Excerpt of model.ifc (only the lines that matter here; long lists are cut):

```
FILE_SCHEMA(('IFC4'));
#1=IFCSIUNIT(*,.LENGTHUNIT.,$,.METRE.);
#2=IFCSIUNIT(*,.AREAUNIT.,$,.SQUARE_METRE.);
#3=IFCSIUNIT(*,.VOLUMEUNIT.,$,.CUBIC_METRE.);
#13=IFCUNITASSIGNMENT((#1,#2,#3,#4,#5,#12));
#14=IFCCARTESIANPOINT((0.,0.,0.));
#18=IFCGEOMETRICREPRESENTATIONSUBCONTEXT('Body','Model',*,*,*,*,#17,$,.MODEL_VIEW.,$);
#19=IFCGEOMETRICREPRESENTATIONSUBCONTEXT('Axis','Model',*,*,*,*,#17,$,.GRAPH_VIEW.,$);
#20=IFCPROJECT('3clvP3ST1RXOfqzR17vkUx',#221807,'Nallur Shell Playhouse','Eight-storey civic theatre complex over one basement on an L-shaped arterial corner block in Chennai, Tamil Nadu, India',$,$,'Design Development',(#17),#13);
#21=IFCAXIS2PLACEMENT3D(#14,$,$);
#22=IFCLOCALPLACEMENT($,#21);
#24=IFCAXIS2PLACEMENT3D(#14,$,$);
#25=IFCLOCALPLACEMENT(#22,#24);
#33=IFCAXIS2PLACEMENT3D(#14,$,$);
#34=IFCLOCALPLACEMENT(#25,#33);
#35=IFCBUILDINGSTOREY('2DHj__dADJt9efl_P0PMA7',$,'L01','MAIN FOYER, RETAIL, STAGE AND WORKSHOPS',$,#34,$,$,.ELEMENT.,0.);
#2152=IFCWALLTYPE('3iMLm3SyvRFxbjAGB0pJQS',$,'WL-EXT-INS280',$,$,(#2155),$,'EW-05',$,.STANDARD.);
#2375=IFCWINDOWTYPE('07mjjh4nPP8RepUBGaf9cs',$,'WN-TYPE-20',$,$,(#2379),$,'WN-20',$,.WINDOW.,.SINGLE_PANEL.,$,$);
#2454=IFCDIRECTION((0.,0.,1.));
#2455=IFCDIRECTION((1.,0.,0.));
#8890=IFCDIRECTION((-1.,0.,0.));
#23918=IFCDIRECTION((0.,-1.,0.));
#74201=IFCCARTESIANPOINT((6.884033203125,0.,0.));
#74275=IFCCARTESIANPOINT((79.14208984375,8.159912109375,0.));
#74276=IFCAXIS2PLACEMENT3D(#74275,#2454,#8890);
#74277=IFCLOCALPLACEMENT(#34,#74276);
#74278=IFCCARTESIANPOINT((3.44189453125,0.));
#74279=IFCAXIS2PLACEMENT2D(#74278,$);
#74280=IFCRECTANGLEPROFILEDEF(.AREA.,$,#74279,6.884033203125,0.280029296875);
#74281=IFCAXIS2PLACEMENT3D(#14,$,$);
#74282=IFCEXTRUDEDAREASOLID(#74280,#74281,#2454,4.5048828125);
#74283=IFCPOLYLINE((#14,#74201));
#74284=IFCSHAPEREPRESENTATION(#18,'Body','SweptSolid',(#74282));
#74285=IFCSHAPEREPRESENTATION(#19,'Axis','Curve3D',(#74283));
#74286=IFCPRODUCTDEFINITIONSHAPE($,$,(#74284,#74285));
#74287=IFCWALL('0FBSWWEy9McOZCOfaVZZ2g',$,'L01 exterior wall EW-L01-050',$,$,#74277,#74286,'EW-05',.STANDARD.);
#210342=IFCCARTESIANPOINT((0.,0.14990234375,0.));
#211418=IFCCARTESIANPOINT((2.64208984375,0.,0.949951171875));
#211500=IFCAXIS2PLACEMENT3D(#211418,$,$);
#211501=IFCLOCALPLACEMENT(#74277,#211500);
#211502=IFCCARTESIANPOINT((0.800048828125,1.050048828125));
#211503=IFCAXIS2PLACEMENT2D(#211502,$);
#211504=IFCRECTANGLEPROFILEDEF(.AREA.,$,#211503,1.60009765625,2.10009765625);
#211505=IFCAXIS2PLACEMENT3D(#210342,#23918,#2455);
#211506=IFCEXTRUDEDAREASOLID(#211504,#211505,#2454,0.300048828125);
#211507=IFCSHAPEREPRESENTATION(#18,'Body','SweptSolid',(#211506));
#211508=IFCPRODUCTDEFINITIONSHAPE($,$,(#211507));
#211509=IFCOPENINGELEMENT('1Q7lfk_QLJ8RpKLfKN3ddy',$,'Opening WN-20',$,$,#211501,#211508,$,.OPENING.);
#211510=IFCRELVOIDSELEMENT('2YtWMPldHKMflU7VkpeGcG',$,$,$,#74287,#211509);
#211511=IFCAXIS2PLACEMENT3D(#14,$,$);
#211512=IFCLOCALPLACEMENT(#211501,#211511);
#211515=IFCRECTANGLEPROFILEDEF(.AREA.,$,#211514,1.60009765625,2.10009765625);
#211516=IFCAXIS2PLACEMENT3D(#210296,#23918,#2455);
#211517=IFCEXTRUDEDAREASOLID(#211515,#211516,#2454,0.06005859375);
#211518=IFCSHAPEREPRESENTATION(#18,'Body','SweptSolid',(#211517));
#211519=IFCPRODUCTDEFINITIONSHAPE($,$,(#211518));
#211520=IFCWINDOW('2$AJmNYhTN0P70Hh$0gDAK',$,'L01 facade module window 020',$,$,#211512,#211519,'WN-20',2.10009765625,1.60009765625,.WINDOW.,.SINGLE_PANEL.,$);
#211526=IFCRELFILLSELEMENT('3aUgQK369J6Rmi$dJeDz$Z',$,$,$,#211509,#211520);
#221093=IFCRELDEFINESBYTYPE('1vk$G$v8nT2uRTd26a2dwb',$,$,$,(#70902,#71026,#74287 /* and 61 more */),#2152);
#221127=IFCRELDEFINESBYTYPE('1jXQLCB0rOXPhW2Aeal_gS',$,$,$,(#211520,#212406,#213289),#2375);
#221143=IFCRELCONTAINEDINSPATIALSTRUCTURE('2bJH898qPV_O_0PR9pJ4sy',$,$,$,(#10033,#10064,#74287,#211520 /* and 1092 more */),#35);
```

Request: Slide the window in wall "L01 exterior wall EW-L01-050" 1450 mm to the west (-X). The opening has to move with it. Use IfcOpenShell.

```python
import ifcopenshell
import ifcopenshell.api.geometry
import ifcopenshell.util.placement
import ifcopenshell.util.unit

model = ifcopenshell.open("model.ifc")
unit_scale = ifcopenshell.util.unit.calculate_unit_scale(model)

window = model.by_guid("2$AJmNYhTN0P70Hh$0gDAK")
opening = window.FillsVoids[0].RelatingOpeningElement
wall = opening.VoidsElements[0].RelatingBuildingElement

wall_matrix = ifcopenshell.util.placement.get_local_placement(wall.ObjectPlacement)
shift = wall_matrix[:3, 0] * 1.45 / unit_scale
before = ifcopenshell.util.placement.get_local_placement(window.ObjectPlacement)[:3, 3].copy()

# The window is placed relative to its opening, so it follows when the opening moves.
matrix = ifcopenshell.util.placement.get_local_placement(opening.ObjectPlacement)
matrix[:3, 3] += shift
ifcopenshell.api.geometry.edit_object_placement(
    model, product=opening, matrix=matrix, is_si=False, should_transform_children=True
)

after = ifcopenshell.util.placement.get_local_placement(window.ObjectPlacement)[:3, 3]
print("window moved by", (after - before).round(3) + 0.0)

model.write("model_v2.ifc")
```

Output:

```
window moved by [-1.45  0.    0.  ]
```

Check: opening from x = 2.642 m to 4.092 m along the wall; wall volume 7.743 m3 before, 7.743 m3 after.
